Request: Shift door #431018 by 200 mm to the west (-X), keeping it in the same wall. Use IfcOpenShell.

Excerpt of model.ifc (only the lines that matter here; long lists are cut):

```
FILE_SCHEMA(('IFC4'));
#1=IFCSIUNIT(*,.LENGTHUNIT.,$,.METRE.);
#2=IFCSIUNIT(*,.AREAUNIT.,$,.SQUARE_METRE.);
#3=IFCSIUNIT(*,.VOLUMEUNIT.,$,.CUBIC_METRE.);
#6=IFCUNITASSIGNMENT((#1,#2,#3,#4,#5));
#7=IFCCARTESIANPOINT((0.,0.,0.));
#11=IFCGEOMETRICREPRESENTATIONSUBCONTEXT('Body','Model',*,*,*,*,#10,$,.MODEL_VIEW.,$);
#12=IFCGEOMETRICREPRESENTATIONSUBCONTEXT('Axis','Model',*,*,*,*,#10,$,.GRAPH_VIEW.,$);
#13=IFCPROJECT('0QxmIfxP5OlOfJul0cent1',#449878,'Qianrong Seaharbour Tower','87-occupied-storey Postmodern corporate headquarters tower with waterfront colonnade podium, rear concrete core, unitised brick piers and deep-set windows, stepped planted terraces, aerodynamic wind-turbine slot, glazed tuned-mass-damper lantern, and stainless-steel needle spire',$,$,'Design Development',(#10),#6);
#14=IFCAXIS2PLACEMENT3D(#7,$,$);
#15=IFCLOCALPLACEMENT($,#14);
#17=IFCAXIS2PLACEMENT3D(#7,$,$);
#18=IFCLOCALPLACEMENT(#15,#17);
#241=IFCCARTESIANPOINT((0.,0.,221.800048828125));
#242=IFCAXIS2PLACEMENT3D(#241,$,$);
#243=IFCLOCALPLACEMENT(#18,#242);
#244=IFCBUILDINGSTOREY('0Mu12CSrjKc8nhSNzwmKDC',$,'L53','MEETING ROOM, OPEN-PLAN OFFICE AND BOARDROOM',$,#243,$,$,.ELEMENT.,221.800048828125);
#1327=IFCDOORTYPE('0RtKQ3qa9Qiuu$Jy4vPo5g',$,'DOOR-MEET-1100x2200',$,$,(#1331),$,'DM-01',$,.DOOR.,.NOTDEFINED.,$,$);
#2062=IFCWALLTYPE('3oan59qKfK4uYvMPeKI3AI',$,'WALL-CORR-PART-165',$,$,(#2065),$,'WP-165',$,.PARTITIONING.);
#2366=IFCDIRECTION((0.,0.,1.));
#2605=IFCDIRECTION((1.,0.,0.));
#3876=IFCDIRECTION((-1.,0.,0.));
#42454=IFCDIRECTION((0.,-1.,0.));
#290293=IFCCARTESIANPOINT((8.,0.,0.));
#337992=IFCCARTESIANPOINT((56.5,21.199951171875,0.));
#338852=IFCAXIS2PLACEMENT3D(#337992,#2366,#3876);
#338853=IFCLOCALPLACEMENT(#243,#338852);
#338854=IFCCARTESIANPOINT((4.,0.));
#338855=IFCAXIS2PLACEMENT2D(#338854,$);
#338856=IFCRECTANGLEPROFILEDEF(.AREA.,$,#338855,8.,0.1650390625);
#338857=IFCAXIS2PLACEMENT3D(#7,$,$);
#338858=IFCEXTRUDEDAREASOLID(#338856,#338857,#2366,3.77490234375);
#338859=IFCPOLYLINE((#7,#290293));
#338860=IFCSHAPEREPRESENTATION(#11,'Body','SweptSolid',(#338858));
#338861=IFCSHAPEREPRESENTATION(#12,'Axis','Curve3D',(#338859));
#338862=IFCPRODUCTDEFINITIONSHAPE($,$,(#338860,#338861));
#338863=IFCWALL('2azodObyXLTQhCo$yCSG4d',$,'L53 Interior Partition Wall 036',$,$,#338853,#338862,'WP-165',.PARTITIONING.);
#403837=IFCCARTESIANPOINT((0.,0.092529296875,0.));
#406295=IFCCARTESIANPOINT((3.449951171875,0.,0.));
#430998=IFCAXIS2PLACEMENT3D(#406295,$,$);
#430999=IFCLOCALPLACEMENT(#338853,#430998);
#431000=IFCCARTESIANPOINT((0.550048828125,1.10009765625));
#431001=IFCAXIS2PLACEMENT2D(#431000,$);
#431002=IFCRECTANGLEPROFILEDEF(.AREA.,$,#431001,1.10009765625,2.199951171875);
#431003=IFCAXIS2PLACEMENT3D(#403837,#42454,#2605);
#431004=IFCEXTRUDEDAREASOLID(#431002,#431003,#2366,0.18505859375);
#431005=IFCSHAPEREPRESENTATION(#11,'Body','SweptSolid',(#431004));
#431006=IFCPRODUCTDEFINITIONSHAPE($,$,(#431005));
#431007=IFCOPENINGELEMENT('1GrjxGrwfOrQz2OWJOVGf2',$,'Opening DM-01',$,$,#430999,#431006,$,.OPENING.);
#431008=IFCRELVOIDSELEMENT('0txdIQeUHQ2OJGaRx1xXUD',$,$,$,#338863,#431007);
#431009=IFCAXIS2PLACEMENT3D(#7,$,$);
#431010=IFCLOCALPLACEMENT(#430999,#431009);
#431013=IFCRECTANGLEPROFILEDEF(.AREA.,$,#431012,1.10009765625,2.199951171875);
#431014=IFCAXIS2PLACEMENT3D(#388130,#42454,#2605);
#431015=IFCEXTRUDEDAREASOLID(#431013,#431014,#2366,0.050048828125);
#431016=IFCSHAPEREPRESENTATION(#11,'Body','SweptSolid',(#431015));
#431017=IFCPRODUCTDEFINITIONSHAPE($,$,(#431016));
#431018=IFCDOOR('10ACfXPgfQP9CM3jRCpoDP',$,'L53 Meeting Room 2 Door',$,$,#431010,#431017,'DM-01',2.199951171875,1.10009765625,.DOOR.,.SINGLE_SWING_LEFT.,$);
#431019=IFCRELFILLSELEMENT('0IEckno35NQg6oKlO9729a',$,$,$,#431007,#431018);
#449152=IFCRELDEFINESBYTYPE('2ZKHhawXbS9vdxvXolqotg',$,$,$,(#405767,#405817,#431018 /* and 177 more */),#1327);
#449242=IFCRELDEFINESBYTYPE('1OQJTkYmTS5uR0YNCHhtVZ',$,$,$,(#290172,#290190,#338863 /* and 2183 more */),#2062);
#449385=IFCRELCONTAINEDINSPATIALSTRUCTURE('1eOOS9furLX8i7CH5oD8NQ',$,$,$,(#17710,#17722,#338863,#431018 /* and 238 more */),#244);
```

```python
import ifcopenshell
import ifcopenshell.api.geometry
import ifcopenshell.util.placement
import ifcopenshell.util.unit

model = ifcopenshell.open("model.ifc")
unit_scale = ifcopenshell.util.unit.calculate_unit_scale(model)

door = model.by_id(431018)
opening = door.FillsVoids[0].RelatingOpeningElement
wall = opening.VoidsElements[0].RelatingBuildingElement

wall_matrix = ifcopenshell.util.placement.get_local_placement(wall.ObjectPlacement)
shift = wall_matrix[:3, 0] * 0.2 / unit_scale
before = ifcopenshell.util.placement.get_local_placement(door.ObjectPlacement)[:3, 3].copy()

# The door is placed relative to its opening, so it follows when the opening moves.
matrix = ifcopenshell.util.placement.get_local_placement(opening.ObjectPlacement)
matrix[:3, 3] += shift
ifcopenshell.api.geometry.edit_object_placement(
    model, product=opening, matrix=matrix, is_si=False, should_transform_children=True
)

after = ifcopenshell.util.placement.get_local_placement(door.ObjectPlacement)[:3, 3]
print("door moved by", (after - before).round(3) + 0.0)

model.write("model_rev.ifc")
```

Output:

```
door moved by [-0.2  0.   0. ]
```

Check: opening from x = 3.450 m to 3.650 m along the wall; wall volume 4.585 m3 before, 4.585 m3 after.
